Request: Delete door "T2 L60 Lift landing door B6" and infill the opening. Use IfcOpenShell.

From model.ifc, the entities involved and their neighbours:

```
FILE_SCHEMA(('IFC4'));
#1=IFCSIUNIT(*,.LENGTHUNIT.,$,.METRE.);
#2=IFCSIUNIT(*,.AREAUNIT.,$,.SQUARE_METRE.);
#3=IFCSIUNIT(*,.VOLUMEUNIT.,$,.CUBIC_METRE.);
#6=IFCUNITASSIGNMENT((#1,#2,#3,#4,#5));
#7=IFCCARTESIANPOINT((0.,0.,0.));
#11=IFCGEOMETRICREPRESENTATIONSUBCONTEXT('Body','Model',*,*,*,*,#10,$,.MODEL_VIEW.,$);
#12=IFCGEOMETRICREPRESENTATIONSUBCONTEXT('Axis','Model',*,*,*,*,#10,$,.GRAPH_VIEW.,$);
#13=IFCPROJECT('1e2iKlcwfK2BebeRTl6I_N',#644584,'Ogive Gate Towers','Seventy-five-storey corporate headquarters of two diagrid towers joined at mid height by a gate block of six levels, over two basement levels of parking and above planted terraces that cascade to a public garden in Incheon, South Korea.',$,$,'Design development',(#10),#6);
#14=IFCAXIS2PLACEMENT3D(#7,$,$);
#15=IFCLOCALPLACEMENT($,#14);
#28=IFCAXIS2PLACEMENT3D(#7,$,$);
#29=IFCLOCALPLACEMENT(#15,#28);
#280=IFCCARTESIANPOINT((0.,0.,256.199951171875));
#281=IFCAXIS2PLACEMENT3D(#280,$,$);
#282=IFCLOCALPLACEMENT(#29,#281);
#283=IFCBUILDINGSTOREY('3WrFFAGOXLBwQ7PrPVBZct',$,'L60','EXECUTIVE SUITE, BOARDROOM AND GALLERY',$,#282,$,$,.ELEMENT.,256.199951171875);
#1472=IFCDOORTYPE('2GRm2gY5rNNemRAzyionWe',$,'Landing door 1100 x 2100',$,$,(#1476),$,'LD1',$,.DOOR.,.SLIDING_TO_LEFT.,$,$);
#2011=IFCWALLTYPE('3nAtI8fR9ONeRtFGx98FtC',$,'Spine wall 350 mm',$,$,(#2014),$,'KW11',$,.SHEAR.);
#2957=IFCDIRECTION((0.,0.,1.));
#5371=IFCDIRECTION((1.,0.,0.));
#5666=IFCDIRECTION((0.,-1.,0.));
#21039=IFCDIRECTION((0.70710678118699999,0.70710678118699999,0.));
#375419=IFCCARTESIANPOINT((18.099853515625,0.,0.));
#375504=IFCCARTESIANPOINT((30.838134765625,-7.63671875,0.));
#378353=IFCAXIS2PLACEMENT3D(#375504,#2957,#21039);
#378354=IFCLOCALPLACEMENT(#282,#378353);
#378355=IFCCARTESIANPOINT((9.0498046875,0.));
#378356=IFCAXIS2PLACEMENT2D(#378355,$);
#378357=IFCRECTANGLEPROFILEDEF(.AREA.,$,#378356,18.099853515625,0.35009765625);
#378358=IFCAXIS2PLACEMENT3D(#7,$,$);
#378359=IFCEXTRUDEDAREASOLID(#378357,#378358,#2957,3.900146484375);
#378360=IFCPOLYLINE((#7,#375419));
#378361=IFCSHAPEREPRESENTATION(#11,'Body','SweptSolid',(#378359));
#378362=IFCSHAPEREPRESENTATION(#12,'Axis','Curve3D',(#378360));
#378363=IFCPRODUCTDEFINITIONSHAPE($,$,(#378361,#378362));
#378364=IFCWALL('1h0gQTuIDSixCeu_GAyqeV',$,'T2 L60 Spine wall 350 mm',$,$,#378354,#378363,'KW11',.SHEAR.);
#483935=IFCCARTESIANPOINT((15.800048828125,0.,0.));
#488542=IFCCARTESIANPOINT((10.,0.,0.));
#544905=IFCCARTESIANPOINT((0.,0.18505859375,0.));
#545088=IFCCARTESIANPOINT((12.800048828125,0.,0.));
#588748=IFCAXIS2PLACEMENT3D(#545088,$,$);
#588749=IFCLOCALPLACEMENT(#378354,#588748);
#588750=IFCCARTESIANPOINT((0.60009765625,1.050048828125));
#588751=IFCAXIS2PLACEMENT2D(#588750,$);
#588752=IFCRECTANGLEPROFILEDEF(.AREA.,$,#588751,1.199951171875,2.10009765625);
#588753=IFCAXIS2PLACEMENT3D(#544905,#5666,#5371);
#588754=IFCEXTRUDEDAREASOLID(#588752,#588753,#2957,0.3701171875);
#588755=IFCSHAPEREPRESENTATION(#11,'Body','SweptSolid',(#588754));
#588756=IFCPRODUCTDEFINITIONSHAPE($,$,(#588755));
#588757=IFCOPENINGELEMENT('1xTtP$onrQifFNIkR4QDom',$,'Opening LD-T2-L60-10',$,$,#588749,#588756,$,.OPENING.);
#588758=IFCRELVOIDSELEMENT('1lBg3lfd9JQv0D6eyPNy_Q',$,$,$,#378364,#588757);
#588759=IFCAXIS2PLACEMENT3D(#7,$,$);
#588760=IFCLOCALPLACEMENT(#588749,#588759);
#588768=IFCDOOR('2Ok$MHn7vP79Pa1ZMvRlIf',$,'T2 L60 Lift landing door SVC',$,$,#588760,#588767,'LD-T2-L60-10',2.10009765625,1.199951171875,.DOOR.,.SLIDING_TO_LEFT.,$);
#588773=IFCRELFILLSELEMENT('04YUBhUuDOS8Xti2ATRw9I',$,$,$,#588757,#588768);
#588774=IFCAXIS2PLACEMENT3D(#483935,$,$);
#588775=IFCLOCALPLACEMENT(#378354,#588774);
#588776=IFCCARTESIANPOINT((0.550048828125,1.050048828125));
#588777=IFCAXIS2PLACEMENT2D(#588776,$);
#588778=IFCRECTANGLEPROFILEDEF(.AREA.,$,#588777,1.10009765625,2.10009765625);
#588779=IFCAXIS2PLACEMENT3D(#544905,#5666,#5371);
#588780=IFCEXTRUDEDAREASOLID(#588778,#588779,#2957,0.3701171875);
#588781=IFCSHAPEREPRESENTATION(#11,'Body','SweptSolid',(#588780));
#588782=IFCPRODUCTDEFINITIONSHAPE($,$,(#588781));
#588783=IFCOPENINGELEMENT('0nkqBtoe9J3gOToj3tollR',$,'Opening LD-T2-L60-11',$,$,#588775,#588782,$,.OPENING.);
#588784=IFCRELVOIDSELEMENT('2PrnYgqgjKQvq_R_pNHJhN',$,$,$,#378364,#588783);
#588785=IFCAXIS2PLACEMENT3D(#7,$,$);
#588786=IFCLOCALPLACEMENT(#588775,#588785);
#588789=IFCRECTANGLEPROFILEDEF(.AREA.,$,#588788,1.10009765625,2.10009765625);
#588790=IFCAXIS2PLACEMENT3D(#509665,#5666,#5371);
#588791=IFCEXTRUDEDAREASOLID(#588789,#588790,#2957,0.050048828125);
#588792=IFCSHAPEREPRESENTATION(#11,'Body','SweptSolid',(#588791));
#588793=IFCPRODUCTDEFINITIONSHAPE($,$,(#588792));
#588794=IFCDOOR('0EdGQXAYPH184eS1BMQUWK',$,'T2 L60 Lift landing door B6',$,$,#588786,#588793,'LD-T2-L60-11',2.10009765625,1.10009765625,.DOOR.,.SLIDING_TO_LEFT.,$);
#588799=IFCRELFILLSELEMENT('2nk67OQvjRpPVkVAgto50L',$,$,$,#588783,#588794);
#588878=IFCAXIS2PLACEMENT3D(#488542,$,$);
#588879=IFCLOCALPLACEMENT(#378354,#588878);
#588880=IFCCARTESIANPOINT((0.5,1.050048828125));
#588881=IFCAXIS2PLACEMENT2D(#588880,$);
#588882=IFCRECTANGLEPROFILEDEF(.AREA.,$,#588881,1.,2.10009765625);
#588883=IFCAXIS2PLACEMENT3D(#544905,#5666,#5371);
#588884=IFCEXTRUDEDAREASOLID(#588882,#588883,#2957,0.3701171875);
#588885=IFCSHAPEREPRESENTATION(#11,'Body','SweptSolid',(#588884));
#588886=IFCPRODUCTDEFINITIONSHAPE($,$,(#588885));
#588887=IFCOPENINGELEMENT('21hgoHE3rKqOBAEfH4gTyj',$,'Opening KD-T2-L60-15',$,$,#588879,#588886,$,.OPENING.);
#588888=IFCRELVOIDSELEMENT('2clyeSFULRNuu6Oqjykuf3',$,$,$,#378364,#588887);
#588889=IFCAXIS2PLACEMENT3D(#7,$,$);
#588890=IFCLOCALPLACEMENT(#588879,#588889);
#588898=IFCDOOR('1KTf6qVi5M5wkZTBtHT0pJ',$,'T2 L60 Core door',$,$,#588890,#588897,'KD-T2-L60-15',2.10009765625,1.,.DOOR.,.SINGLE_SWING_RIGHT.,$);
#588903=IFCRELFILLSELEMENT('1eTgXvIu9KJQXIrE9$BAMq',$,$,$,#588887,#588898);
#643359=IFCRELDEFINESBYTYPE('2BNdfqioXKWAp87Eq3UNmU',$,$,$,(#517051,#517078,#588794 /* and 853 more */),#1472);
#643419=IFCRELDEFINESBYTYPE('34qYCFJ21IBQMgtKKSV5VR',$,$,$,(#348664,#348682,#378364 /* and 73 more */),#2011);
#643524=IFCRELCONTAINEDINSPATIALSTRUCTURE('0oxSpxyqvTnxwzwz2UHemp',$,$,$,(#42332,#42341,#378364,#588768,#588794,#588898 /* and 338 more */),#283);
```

```python
import ifcopenshell
import ifcopenshell.api.feature
import ifcopenshell.api.root
import ifcopenshell.geom
import ifcopenshell.util.shape

model = ifcopenshell.open("model.ifc")
settings = ifcopenshell.geom.settings()


def volume(element):
    """Net volume in cubic metres, openings subtracted."""
    shape = ifcopenshell.geom.create_shape(settings, element)
    return ifcopenshell.util.shape.get_volume(shape.geometry)


door = model.by_guid("0EdGQXAYPH184eS1BMQUWK")
opening = door.FillsVoids[0].RelatingOpeningElement
wall = opening.VoidsElements[0].RelatingBuildingElement
before = volume(wall)

ifcopenshell.api.root.remove_product(model, product=door)
ifcopenshell.api.feature.remove_feature(model, feature=opening)

after = volume(wall)

print(f"wall volume {before:.3f} -> {after:.3f} m3")

model.write("model_edited.ifc")
```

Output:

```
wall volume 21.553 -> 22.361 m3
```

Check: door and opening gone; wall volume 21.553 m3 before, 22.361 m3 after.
